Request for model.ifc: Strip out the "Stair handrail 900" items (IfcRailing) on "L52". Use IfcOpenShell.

First a look at what the model holds.

```python
import ifcopenshell
import ifcopenshell.util.element

model = ifcopenshell.open("model.ifc")
print(model.schema)
storey = next(s for s in model.by_type("IfcBuildingStorey") if s.Name == "L52")
railings = [e for e in ifcopenshell.util.element.get_decomposition(storey) if e.is_a("IfcRailing")]
seen = {}
for e in railings:
    element_type = ifcopenshell.util.element.get_type(e)
    name = element_type.Name if element_type not in (None, e) else None
    seen[name] = seen.get(name, 0) + 1
for name, count in sorted(seen.items(), key=str):
    print(count, "x", name)
```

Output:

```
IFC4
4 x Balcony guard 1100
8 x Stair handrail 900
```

```python
import ifcopenshell
import ifcopenshell.api.root
import ifcopenshell.util.element

model = ifcopenshell.open("model.ifc")

storey = next(s for s in model.by_type("IfcBuildingStorey") if s.Name == "L52")
railings = [e for e in ifcopenshell.util.element.get_decomposition(storey) if e.is_a("IfcRailing")]
targets = [e for e in railings if (t := ifcopenshell.util.element.get_type(e)) not in (None, e) and t.Name == "Stair handrail 900"]

for e in targets:
    ifcopenshell.api.root.remove_product(model, product=e)
print(len(targets), "removed")

model.write("model-out.ifc")
```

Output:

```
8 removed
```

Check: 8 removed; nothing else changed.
